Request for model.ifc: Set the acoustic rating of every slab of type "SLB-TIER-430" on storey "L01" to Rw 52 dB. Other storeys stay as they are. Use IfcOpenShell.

First a look at what the model holds.

```python
import ifcopenshell
import ifcopenshell.util.element

model = ifcopenshell.open("model.ifc")
print(model.schema)
storey = next(s for s in model.by_type("IfcBuildingStorey") if s.Name == "L01")
slabs = [e for e in ifcopenshell.util.element.get_decomposition(storey) if e.is_a("IfcSlab")]
seen = {}
for e in slabs:
    element_type = ifcopenshell.util.element.get_type(e)
    key = (element_type.Name if element_type != e and element_type else None, ifcopenshell.util.element.get_pset(e, "Pset_SlabCommon", "AcousticRating"))
    seen[key] = seen.get(key, 0) + 1
for (name, value), count in sorted(seen.items(), key=str):
    print(count, "x", name, "|", value)
```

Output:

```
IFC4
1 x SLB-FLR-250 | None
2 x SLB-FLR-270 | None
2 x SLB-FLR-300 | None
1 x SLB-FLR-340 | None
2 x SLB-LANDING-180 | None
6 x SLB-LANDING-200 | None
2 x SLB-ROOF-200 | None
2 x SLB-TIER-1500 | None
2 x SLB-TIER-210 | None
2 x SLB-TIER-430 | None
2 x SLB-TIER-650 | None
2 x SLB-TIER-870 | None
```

```python
import ifcopenshell
import ifcopenshell.api.pset
import ifcopenshell.util.element

model = ifcopenshell.open("model.ifc")

storey = next(s for s in model.by_type("IfcBuildingStorey") if s.Name == "L01")
slabs = [e for e in ifcopenshell.util.element.get_decomposition(storey) if e.is_a("IfcSlab")]

count = 0
for e in slabs:
    element_type = ifcopenshell.util.element.get_type(e)
    if element_type in (None, e) or element_type.Name != "SLB-TIER-430":
        continue
    # add_pset returns the element's existing set when there is one.
    pset = ifcopenshell.api.pset.add_pset(model, product=e, name="Pset_SlabCommon")
    ifcopenshell.api.pset.edit_pset(model, pset=pset, properties={"AcousticRating": "Rw 52 dB"})
    count += 1

print(count, "slabs updated")

model.write("model-out.ifc")
```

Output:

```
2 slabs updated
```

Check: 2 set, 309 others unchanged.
